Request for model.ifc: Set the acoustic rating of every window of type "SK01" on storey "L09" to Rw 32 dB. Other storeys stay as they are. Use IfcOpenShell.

First a look at what the model holds.

```python
import ifcopenshell
import ifcopenshell.util.element

model = ifcopenshell.open("model.ifc")
print(model.schema)
storey = next(s for s in model.by_type("IfcBuildingStorey") if s.Name == "L09")
windows = [e for e in ifcopenshell.util.element.get_decomposition(storey) if e.is_a("IfcWindow")]
seen = {}
for e in windows:
    element_type = ifcopenshell.util.element.get_type(e)
    key = (element_type.Name if element_type != e and element_type else None, ifcopenshell.util.element.get_pset(e, "Pset_WindowCommon", "AcousticRating"))
    seen[key] = seen.get(key, 0) + 1
for (name, value), count in sorted(seen.items(), key=str):
    print(count, "x", name, "|", value)
```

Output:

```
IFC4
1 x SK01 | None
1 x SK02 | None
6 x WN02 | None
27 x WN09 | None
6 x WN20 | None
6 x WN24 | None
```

```python
import ifcopenshell
import ifcopenshell.api.pset
import ifcopenshell.util.element

model = ifcopenshell.open("model.ifc")

storey = next(s for s in model.by_type("IfcBuildingStorey") if s.Name == "L09")
windows = [e for e in ifcopenshell.util.element.get_decomposition(storey) if e.is_a("IfcWindow")]

count = 0
for e in windows:
    element_type = ifcopenshell.util.element.get_type(e)
    if element_type in (None, e) or element_type.Name != "SK01":
        continue
    # add_pset returns the element's existing set when there is one.
    pset = ifcopenshell.api.pset.add_pset(model, product=e, name="Pset_WindowCommon")
    ifcopenshell.api.pset.edit_pset(model, pset=pset, properties={"AcousticRating": "Rw 32 dB"})
    count += 1

print(count, "windows updated")

model.write("model_rev.ifc")
```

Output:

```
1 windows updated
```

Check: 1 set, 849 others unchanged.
